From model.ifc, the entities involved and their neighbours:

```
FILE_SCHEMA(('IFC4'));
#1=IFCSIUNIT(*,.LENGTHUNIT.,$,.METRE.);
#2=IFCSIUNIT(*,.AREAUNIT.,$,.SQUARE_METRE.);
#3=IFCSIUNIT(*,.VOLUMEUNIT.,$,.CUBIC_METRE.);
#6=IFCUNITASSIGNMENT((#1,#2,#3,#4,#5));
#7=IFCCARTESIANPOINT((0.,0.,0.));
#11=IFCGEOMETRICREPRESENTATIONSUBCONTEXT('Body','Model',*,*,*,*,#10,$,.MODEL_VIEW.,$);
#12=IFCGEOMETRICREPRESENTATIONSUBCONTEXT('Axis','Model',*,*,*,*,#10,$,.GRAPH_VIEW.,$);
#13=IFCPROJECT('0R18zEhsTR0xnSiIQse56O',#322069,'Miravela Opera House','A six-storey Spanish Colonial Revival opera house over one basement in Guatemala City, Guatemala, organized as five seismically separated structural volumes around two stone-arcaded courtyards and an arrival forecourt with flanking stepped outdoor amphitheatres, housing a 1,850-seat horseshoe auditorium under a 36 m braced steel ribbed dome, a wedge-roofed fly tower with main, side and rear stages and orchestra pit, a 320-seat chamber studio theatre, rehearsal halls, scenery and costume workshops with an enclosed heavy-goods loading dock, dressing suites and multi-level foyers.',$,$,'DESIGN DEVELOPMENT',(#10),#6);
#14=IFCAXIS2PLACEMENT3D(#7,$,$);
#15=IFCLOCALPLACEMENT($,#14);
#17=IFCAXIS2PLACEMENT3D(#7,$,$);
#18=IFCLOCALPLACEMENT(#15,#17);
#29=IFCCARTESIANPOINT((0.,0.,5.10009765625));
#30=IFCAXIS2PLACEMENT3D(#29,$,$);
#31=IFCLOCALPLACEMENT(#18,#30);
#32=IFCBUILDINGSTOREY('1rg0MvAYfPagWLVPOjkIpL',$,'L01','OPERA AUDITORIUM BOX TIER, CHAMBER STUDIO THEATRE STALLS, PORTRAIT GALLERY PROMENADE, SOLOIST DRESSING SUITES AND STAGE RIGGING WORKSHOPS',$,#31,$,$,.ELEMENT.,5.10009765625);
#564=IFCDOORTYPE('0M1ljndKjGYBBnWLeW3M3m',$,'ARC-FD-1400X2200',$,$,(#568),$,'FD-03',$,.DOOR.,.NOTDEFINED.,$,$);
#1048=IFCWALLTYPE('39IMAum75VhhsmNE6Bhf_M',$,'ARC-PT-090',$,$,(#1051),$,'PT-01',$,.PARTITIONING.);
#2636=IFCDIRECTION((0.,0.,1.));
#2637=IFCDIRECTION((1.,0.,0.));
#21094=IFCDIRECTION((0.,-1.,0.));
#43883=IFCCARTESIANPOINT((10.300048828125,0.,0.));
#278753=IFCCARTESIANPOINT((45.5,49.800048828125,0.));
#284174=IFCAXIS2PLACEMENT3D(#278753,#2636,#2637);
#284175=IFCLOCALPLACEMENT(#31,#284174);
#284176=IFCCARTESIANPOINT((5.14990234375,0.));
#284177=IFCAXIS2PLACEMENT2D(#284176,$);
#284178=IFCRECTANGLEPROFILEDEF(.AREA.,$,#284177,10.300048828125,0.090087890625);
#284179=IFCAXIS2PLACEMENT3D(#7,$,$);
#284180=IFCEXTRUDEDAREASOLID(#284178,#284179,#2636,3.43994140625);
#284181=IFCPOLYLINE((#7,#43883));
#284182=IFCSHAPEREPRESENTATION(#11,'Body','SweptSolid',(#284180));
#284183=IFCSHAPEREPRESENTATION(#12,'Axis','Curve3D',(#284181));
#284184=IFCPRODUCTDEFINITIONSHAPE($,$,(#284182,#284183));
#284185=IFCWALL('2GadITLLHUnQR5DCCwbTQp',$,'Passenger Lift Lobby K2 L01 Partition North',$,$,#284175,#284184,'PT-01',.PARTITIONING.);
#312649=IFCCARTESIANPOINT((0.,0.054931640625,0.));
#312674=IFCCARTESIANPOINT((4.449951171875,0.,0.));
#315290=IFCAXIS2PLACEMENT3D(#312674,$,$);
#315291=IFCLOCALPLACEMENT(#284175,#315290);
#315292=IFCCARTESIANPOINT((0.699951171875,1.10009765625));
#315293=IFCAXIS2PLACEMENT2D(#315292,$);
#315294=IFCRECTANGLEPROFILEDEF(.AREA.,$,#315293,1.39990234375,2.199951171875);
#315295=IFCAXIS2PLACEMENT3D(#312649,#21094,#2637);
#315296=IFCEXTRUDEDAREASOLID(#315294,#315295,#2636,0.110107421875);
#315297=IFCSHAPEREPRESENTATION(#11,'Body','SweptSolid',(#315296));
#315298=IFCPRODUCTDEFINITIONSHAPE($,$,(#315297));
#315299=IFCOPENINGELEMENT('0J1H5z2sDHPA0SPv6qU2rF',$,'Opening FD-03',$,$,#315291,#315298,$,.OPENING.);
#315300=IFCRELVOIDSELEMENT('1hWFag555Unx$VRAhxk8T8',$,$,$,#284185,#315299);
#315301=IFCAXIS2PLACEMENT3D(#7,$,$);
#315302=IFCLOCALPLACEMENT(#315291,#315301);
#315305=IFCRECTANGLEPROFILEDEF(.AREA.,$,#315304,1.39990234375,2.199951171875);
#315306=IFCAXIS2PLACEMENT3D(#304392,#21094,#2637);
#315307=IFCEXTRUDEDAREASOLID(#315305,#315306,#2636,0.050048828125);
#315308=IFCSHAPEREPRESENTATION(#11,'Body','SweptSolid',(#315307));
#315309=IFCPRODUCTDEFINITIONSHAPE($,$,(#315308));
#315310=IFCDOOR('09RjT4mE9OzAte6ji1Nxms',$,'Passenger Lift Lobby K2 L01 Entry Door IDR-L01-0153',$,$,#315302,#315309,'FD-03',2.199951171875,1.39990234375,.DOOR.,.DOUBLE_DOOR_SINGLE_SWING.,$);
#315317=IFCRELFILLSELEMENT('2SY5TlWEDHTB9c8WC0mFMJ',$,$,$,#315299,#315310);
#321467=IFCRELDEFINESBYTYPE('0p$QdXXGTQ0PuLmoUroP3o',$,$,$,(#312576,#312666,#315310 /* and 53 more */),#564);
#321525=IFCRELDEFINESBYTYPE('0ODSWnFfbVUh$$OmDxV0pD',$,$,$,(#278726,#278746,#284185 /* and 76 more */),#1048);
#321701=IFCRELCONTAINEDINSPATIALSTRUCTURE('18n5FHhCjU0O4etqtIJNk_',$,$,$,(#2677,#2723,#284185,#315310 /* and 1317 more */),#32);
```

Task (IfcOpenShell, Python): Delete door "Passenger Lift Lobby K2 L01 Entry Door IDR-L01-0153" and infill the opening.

```python
import ifcopenshell
import ifcopenshell.api.feature
import ifcopenshell.api.root
import ifcopenshell.geom
import ifcopenshell.util.shape

model = ifcopenshell.open("model.ifc")
settings = ifcopenshell.geom.settings()


def volume(element):
    """Net volume in cubic metres, openings subtracted."""
    shape = ifcopenshell.geom.create_shape(settings, element)
    return ifcopenshell.util.shape.get_volume(shape.geometry)


door = model.by_guid("09RjT4mE9OzAte6ji1Nxms")
opening = door.FillsVoids[0].RelatingOpeningElement
wall = opening.VoidsElements[0].RelatingBuildingElement
before = volume(wall)

ifcopenshell.api.root.remove_product(model, product=door)
ifcopenshell.api.feature.remove_feature(model, feature=opening)

after = volume(wall)

print(f"wall volume {before:.3f} -> {after:.3f} m3")

model.write("model_rev.ifc")
```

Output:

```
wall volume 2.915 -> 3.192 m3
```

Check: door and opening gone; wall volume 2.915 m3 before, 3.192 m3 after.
